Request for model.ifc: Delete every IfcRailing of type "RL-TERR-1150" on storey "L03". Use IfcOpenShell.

First a look at what the model holds.

```python
import ifcopenshell
import ifcopenshell.util.element

model = ifcopenshell.open("model.ifc")
print(model.schema)
storey = next(s for s in model.by_type("IfcBuildingStorey") if s.Name == "L03")
railings = [e for e in ifcopenshell.util.element.get_decomposition(storey) if e.is_a("IfcRailing")]
seen = {}
for e in railings:
    element_type = ifcopenshell.util.element.get_type(e)
    name = element_type.Name if element_type not in (None, e) else None
    seen[name] = seen.get(name, 0) + 1
for name, count in sorted(seen.items(), key=str):
    print(count, "x", name)
```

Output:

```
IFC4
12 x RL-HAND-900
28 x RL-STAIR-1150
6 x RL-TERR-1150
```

```python
import ifcopenshell
import ifcopenshell.api.root
import ifcopenshell.util.element

model = ifcopenshell.open("model.ifc")

storey = next(s for s in model.by_type("IfcBuildingStorey") if s.Name == "L03")
railings = [e for e in ifcopenshell.util.element.get_decomposition(storey) if e.is_a("IfcRailing")]
targets = [e for e in railings if (t := ifcopenshell.util.element.get_type(e)) not in (None, e) and t.Name == "RL-TERR-1150"]

for e in targets:
    ifcopenshell.api.root.remove_product(model, product=e)
print(len(targets), "removed")

model.write("model_rev.ifc")
```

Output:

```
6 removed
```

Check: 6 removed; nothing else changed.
